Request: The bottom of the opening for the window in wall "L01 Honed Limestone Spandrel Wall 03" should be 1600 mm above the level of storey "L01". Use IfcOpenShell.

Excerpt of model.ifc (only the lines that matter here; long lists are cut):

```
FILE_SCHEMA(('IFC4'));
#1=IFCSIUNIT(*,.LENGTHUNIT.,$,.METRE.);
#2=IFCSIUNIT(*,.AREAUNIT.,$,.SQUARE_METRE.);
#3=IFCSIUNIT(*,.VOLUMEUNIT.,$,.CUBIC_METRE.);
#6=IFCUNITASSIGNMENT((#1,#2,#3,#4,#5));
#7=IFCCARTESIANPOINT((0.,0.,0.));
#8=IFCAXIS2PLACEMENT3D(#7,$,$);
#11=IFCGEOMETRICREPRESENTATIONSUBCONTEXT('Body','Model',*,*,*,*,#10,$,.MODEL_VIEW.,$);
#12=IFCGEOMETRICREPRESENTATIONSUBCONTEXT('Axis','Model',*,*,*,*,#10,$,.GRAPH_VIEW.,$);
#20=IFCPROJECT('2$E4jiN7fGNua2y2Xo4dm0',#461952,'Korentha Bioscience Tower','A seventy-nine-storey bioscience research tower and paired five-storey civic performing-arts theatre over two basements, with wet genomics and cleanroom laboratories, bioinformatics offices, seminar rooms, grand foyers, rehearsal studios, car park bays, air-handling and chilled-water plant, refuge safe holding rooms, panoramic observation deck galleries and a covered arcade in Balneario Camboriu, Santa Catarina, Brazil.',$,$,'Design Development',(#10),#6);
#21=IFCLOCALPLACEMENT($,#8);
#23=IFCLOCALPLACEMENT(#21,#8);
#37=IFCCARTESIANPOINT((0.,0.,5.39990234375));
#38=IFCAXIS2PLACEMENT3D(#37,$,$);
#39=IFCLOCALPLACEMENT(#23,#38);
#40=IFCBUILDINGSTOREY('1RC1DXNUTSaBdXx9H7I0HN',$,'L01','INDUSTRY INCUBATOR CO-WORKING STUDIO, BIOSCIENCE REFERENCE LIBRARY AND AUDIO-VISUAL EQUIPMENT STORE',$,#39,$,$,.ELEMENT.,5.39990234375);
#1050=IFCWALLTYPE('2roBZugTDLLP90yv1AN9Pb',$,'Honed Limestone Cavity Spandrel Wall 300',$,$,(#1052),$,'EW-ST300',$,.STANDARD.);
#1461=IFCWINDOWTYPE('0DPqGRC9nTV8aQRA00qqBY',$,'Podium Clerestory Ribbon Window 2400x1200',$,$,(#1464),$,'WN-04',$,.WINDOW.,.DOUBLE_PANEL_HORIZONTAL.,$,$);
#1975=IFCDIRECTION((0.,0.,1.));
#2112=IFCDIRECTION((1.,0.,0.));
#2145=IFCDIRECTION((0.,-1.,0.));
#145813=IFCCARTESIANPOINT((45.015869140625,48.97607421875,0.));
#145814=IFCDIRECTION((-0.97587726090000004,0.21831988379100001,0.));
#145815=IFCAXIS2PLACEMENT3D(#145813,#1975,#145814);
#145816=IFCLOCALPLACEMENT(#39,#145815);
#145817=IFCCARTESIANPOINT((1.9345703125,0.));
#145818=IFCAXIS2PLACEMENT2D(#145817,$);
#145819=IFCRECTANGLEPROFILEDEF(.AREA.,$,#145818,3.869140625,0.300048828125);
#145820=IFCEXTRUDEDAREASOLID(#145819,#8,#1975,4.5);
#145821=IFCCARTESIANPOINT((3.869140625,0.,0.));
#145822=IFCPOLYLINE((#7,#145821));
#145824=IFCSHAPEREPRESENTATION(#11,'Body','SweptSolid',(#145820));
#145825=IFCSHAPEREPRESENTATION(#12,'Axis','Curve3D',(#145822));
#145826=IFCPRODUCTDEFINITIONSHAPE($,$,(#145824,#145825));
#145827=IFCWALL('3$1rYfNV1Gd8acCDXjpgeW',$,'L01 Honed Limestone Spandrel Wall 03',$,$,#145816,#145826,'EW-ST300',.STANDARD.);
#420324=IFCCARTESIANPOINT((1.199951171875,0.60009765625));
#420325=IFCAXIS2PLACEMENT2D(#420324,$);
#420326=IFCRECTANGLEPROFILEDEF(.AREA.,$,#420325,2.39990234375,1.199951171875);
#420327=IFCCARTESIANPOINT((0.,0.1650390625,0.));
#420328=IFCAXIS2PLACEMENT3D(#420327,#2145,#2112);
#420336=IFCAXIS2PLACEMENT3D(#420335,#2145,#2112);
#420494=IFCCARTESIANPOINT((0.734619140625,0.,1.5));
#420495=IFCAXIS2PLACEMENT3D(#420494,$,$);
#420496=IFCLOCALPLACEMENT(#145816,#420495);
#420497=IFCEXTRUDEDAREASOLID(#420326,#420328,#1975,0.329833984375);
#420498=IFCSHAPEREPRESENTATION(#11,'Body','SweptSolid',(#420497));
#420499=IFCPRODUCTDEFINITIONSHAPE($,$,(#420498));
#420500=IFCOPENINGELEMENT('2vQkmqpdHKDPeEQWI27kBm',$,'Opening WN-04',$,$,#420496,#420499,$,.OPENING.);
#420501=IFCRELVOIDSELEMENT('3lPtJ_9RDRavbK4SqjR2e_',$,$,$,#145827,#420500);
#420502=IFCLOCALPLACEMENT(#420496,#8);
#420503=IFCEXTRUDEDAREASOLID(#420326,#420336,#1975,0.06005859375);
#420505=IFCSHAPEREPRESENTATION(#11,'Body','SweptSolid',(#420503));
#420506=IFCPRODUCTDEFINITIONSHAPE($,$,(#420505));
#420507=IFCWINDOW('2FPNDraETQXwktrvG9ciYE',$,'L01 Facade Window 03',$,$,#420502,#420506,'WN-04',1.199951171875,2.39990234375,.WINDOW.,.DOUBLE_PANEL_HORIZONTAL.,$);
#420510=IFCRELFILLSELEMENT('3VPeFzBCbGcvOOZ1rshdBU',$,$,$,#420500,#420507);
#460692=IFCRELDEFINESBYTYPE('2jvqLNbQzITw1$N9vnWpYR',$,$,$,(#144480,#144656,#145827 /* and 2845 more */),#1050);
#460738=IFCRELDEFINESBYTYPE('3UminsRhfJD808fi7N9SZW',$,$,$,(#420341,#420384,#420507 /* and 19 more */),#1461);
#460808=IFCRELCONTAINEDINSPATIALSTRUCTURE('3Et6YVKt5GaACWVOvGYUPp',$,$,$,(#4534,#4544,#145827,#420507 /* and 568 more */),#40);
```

```python
import numpy as np
import ifcopenshell
import ifcopenshell.api.geometry
import ifcopenshell.geom
import ifcopenshell.util.element
import ifcopenshell.util.placement
import ifcopenshell.util.shape
import ifcopenshell.util.unit

model = ifcopenshell.open("model.ifc")
unit_scale = ifcopenshell.util.unit.calculate_unit_scale(model)

window = model.by_guid("2FPNDraETQXwktrvG9ciYE")
opening = window.FillsVoids[0].RelatingOpeningElement
storey = ifcopenshell.util.element.get_container(window, ifc_class="IfcBuildingStorey")
level = ifcopenshell.util.placement.get_local_placement(storey.ObjectPlacement)[2, 3]

# The opening's origin need not be at the sill, so measure its lowest point.
shape = ifcopenshell.geom.create_shape(ifcopenshell.geom.settings(), opening)
bottom = ifcopenshell.util.shape.get_shape_bottom_elevation(shape, shape.geometry) / unit_scale
dz = level + 1.6 / unit_scale - bottom

shift = np.array([0.0, 0.0, dz])
# The window is placed relative to its opening, so it follows when the opening moves.
matrix = ifcopenshell.util.placement.get_local_placement(opening.ObjectPlacement)
matrix[:3, 3] += shift
ifcopenshell.api.geometry.edit_object_placement(
    model, product=opening, matrix=matrix, is_si=False, should_transform_children=True
)

print(f"moved by {dz * unit_scale:+.3f} m")

model.write("model_edited.ifc")
```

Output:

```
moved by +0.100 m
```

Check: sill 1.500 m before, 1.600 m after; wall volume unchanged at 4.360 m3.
